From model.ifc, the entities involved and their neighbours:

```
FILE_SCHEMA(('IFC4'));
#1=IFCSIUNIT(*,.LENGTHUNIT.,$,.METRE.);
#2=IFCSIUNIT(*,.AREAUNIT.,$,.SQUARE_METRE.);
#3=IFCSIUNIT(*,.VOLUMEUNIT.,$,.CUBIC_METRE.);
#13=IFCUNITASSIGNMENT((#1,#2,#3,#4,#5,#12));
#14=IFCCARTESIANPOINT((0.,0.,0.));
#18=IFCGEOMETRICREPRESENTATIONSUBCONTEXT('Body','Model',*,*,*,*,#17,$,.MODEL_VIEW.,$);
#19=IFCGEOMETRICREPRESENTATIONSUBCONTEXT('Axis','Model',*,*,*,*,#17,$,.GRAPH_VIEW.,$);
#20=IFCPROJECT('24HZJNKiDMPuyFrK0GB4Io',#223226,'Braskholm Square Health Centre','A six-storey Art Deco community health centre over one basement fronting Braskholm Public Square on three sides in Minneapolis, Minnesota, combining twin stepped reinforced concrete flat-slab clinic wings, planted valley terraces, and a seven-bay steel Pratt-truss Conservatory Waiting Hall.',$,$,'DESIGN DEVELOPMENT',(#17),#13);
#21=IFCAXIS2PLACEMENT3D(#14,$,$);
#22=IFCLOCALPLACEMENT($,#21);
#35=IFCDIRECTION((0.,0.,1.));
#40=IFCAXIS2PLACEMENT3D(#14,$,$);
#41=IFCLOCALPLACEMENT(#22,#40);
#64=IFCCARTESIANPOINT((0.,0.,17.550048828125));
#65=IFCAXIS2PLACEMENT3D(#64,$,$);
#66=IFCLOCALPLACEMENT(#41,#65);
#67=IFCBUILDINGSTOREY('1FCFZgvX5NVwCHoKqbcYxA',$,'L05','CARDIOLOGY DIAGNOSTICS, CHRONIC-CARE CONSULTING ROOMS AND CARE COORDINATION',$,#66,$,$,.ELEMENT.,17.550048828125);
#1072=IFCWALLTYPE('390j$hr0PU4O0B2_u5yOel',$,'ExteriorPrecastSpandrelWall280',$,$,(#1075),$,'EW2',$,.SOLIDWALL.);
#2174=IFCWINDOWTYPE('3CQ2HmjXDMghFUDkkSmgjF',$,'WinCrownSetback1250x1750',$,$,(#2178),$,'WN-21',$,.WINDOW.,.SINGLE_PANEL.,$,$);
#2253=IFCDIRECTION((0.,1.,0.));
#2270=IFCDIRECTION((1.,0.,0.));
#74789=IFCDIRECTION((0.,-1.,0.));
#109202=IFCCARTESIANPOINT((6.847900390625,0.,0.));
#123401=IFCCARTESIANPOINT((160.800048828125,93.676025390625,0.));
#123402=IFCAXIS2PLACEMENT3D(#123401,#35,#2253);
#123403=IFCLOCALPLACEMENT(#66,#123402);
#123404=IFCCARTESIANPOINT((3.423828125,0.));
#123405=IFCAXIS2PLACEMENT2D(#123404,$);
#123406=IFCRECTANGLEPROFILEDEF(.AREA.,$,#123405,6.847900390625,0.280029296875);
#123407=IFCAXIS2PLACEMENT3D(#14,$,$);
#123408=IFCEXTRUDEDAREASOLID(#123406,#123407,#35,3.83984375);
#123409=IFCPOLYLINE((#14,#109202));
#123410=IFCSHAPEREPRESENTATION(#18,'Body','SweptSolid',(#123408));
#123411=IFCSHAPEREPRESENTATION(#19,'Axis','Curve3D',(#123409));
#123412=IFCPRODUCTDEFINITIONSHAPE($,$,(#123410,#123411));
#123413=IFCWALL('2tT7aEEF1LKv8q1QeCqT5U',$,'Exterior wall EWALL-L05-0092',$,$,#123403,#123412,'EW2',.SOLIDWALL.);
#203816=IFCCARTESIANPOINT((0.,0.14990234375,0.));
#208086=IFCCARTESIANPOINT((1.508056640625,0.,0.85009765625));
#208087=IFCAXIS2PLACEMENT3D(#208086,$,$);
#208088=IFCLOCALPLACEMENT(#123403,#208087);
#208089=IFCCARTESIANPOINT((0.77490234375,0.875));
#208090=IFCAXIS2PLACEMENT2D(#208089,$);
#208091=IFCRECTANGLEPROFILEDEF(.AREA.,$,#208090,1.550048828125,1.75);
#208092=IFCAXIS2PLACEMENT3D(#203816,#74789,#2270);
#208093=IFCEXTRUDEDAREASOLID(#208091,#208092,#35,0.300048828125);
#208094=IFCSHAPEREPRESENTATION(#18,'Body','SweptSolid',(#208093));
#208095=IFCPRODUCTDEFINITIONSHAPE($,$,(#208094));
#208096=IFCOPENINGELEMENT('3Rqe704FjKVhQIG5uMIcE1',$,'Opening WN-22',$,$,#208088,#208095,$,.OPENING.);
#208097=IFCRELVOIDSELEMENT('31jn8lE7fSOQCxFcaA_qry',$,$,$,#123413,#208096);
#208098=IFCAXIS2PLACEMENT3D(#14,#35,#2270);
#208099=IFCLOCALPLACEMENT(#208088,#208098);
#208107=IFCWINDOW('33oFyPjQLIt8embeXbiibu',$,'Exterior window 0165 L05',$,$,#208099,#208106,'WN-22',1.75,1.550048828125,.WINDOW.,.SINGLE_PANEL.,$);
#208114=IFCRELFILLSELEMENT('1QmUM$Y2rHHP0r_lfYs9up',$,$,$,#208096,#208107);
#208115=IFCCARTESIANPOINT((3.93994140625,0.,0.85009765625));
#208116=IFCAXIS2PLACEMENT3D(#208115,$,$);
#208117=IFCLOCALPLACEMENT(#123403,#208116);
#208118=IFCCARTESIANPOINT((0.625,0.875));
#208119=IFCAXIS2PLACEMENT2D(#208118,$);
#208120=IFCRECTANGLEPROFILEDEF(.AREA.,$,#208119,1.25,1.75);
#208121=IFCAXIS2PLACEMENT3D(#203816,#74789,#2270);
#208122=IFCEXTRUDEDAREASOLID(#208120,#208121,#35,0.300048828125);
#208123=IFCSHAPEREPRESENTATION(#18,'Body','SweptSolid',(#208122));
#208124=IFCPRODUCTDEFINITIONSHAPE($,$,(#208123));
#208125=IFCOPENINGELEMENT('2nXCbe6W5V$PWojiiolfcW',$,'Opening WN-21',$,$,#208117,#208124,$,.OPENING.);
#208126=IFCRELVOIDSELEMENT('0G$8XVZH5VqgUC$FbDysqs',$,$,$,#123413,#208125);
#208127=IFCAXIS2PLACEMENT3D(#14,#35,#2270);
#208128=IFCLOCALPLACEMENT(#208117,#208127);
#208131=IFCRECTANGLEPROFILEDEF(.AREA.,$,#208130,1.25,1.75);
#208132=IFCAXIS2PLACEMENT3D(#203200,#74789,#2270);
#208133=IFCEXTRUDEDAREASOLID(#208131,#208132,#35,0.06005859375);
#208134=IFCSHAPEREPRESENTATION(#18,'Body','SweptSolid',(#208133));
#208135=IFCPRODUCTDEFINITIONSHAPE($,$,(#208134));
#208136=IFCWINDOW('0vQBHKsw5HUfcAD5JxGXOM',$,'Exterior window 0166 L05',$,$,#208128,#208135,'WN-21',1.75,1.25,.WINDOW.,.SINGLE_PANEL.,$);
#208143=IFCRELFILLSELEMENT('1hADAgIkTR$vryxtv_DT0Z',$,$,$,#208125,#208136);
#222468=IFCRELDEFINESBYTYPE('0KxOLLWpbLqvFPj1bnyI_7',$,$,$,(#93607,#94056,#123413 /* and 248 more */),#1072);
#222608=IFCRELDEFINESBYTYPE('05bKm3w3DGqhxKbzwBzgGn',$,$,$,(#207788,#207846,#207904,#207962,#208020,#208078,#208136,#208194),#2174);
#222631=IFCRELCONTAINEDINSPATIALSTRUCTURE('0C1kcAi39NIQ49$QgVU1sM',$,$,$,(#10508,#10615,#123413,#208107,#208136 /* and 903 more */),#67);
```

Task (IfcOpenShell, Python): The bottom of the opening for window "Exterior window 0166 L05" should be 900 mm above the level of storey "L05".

```python
import numpy as np
import ifcopenshell
import ifcopenshell.api.geometry
import ifcopenshell.geom
import ifcopenshell.util.element
import ifcopenshell.util.placement
import ifcopenshell.util.shape
import ifcopenshell.util.unit

model = ifcopenshell.open("model.ifc")
unit_scale = ifcopenshell.util.unit.calculate_unit_scale(model)

window = model.by_id(208136)
opening = window.FillsVoids[0].RelatingOpeningElement
storey = ifcopenshell.util.element.get_container(window, ifc_class="IfcBuildingStorey")
level = ifcopenshell.util.placement.get_local_placement(storey.ObjectPlacement)[2, 3]

# The opening's origin need not be at the sill, so measure its lowest point.
shape = ifcopenshell.geom.create_shape(ifcopenshell.geom.settings(), opening)
bottom = ifcopenshell.util.shape.get_shape_bottom_elevation(shape, shape.geometry) / unit_scale
dz = level + 0.9 / unit_scale - bottom

shift = np.array([0.0, 0.0, dz])
# The window is placed relative to its opening, so it follows when the opening moves.
matrix = ifcopenshell.util.placement.get_local_placement(opening.ObjectPlacement)
matrix[:3, 3] += shift
ifcopenshell.api.geometry.edit_object_placement(
    model, product=opening, matrix=matrix, is_si=False, should_transform_children=True
)

print(f"moved by {dz * unit_scale:+.3f} m")

model.write("model_updated.ifc")
```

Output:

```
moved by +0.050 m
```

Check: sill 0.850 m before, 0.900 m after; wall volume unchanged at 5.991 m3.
